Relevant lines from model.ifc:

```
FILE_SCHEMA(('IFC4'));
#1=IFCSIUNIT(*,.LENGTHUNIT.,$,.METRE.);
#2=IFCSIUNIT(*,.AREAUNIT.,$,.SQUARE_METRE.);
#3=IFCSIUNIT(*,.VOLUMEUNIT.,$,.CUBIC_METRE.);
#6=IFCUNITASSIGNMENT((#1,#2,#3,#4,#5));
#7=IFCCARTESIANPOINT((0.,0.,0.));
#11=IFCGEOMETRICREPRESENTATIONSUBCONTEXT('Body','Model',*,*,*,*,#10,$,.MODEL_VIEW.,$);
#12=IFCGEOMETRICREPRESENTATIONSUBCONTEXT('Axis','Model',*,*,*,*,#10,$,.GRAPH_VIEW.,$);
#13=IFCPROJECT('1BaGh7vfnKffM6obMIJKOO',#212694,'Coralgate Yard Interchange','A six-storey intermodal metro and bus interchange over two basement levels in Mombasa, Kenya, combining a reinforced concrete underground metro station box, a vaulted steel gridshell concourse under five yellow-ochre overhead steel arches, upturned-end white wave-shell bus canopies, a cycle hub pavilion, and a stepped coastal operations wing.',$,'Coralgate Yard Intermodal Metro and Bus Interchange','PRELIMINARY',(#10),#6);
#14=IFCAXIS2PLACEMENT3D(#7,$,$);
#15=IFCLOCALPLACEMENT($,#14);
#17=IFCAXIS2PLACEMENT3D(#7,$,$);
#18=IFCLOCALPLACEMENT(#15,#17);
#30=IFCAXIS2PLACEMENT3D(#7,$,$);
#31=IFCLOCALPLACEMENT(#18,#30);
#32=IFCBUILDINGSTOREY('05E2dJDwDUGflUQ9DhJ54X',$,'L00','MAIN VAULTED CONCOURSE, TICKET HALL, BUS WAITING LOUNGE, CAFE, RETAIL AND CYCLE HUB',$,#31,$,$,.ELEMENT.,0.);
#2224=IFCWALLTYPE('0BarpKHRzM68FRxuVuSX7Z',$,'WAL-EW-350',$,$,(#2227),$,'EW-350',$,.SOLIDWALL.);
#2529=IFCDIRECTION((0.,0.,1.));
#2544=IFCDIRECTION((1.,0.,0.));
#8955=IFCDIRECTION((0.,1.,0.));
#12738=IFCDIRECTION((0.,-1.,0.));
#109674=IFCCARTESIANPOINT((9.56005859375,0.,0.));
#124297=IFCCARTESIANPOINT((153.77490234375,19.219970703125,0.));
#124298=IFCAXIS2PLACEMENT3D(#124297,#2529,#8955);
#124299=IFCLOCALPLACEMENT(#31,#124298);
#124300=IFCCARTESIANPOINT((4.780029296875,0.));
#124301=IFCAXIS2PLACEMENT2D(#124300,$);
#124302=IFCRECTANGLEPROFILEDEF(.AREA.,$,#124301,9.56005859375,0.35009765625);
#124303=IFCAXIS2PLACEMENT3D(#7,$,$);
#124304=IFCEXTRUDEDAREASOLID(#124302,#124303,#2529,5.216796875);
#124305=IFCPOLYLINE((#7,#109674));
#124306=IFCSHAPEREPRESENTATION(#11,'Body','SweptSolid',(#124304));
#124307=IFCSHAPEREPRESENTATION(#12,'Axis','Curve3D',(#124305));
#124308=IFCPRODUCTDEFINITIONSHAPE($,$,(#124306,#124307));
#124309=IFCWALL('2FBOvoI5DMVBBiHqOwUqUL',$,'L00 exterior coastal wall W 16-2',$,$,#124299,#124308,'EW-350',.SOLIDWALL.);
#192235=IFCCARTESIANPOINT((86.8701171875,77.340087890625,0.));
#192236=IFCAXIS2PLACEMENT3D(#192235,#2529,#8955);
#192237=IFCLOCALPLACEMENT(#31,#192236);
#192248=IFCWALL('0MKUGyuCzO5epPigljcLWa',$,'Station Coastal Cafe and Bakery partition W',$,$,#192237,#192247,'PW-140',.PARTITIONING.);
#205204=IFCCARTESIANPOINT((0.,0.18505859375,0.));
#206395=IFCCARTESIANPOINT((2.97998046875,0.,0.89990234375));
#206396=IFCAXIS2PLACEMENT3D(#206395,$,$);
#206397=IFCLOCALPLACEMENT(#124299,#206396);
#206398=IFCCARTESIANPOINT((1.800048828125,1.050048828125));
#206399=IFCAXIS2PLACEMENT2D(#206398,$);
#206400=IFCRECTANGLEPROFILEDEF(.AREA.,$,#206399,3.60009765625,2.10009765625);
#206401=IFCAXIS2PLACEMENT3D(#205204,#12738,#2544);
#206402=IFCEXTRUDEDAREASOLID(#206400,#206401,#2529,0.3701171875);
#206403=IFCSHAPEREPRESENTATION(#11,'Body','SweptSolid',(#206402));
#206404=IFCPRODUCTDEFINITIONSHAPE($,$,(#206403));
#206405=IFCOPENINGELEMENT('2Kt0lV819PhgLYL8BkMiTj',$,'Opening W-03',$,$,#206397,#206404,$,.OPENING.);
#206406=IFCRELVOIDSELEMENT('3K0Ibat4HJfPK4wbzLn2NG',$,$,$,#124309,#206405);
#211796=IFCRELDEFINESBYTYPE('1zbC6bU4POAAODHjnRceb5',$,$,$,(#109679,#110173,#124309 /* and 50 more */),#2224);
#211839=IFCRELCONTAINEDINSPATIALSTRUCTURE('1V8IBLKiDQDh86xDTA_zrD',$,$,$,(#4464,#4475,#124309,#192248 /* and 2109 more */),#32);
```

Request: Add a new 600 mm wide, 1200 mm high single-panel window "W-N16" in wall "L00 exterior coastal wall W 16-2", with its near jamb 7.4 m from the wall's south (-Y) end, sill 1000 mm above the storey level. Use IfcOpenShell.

```python
import numpy as np
import ifcopenshell
import ifcopenshell.api.feature
import ifcopenshell.api.geometry
import ifcopenshell.api.root
import ifcopenshell.api.spatial
import ifcopenshell.geom
import ifcopenshell.util.element
import ifcopenshell.util.placement
import ifcopenshell.util.representation
import ifcopenshell.util.shape
import ifcopenshell.util.unit

model = ifcopenshell.open("model.ifc")
unit_scale = ifcopenshell.util.unit.calculate_unit_scale(model)
settings = ifcopenshell.geom.settings()


def volume(element):
    """Net volume in cubic metres, openings subtracted."""
    shape = ifcopenshell.geom.create_shape(settings, element)
    return ifcopenshell.util.shape.get_volume(shape.geometry)


wall = model.by_id(124309)
storey = ifcopenshell.util.element.get_container(wall, ifc_class="IfcBuildingStorey")
context = ifcopenshell.util.representation.get_context(model, "Model", "Body", "MODEL_VIEW")
before = volume(wall)

width, height, from_end, sill = 0.6, 1.2, 7.4, 1  # metres

# The wall runs along its own X axis, and the end named is its -X end.
wall_shape = ifcopenshell.geom.create_shape(settings, wall)
x, y, z = ifcopenshell.util.shape.get_vertices(wall_shape.geometry).T
start = x.min() + from_end
face, thickness = float(y.min()), float(y.max() - y.min())
wall_matrix = ifcopenshell.util.placement.get_local_placement(wall.ObjectPlacement)
level = ifcopenshell.util.placement.get_local_placement(storey.ObjectPlacement)[2, 3]


def in_wall(x, y):
    """Placement at x, y metres in the wall's axes, at sill height."""
    matrix = wall_matrix.copy()
    matrix[:, 3] = wall_matrix @ np.array([x / unit_scale, y / unit_scale, 0.0, 1.0])
    matrix[2, 3] = level + sill / unit_scale
    return matrix


# Opening: a box that overshoots both wall faces by 50 mm.
opening = ifcopenshell.api.root.create_entity(model, ifc_class="IfcOpeningElement", predefined_type="OPENING")
box = ifcopenshell.api.geometry.add_wall_representation(
    model, context=context, length=width, height=height, thickness=thickness + 0.1
)
ifcopenshell.api.geometry.assign_representation(model, product=opening, representation=box)
ifcopenshell.api.geometry.edit_object_placement(model, product=opening, matrix=in_wall(start, face - 0.05), is_si=False)
ifcopenshell.api.feature.add_feature(model, feature=opening, element=wall)

window = ifcopenshell.api.root.create_entity(model, ifc_class="IfcWindow", name="W-N16", predefined_type="WINDOW")
window.OverallWidth, window.OverallHeight = width / unit_scale, height / unit_scale
window.PartitioningType = "SINGLE_PANEL"
body = ifcopenshell.api.geometry.add_window_representation(
    model,
    context=context,
    overall_width=window.OverallWidth,
    overall_height=window.OverallHeight,
    partition_type="SINGLE_PANEL",
)
ifcopenshell.api.geometry.assign_representation(model, product=window, representation=body)
ifcopenshell.api.spatial.assign_container(model, products=[window], relating_structure=storey)
ifcopenshell.api.feature.add_filling(model, opening=opening, element=window)

# Centre the window in the wall's thickness.
ifcopenshell.api.geometry.edit_object_placement(model, product=window, matrix=in_wall(start, face), is_si=False)
window_shape = ifcopenshell.geom.create_shape(settings, window)
depth = ifcopenshell.util.shape.get_vertices(window_shape.geometry)[:, 1]
offset = face + thickness / 2 - (depth.min() + depth.max()) / 2
ifcopenshell.api.geometry.edit_object_placement(model, product=window, matrix=in_wall(start, offset), is_si=False)

after = volume(wall)

print(f"wall volume {before:.3f} -> {after:.3f} m3")

model.write("model_v2.ifc")
```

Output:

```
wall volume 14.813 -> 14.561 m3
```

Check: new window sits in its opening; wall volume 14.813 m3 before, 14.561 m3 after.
